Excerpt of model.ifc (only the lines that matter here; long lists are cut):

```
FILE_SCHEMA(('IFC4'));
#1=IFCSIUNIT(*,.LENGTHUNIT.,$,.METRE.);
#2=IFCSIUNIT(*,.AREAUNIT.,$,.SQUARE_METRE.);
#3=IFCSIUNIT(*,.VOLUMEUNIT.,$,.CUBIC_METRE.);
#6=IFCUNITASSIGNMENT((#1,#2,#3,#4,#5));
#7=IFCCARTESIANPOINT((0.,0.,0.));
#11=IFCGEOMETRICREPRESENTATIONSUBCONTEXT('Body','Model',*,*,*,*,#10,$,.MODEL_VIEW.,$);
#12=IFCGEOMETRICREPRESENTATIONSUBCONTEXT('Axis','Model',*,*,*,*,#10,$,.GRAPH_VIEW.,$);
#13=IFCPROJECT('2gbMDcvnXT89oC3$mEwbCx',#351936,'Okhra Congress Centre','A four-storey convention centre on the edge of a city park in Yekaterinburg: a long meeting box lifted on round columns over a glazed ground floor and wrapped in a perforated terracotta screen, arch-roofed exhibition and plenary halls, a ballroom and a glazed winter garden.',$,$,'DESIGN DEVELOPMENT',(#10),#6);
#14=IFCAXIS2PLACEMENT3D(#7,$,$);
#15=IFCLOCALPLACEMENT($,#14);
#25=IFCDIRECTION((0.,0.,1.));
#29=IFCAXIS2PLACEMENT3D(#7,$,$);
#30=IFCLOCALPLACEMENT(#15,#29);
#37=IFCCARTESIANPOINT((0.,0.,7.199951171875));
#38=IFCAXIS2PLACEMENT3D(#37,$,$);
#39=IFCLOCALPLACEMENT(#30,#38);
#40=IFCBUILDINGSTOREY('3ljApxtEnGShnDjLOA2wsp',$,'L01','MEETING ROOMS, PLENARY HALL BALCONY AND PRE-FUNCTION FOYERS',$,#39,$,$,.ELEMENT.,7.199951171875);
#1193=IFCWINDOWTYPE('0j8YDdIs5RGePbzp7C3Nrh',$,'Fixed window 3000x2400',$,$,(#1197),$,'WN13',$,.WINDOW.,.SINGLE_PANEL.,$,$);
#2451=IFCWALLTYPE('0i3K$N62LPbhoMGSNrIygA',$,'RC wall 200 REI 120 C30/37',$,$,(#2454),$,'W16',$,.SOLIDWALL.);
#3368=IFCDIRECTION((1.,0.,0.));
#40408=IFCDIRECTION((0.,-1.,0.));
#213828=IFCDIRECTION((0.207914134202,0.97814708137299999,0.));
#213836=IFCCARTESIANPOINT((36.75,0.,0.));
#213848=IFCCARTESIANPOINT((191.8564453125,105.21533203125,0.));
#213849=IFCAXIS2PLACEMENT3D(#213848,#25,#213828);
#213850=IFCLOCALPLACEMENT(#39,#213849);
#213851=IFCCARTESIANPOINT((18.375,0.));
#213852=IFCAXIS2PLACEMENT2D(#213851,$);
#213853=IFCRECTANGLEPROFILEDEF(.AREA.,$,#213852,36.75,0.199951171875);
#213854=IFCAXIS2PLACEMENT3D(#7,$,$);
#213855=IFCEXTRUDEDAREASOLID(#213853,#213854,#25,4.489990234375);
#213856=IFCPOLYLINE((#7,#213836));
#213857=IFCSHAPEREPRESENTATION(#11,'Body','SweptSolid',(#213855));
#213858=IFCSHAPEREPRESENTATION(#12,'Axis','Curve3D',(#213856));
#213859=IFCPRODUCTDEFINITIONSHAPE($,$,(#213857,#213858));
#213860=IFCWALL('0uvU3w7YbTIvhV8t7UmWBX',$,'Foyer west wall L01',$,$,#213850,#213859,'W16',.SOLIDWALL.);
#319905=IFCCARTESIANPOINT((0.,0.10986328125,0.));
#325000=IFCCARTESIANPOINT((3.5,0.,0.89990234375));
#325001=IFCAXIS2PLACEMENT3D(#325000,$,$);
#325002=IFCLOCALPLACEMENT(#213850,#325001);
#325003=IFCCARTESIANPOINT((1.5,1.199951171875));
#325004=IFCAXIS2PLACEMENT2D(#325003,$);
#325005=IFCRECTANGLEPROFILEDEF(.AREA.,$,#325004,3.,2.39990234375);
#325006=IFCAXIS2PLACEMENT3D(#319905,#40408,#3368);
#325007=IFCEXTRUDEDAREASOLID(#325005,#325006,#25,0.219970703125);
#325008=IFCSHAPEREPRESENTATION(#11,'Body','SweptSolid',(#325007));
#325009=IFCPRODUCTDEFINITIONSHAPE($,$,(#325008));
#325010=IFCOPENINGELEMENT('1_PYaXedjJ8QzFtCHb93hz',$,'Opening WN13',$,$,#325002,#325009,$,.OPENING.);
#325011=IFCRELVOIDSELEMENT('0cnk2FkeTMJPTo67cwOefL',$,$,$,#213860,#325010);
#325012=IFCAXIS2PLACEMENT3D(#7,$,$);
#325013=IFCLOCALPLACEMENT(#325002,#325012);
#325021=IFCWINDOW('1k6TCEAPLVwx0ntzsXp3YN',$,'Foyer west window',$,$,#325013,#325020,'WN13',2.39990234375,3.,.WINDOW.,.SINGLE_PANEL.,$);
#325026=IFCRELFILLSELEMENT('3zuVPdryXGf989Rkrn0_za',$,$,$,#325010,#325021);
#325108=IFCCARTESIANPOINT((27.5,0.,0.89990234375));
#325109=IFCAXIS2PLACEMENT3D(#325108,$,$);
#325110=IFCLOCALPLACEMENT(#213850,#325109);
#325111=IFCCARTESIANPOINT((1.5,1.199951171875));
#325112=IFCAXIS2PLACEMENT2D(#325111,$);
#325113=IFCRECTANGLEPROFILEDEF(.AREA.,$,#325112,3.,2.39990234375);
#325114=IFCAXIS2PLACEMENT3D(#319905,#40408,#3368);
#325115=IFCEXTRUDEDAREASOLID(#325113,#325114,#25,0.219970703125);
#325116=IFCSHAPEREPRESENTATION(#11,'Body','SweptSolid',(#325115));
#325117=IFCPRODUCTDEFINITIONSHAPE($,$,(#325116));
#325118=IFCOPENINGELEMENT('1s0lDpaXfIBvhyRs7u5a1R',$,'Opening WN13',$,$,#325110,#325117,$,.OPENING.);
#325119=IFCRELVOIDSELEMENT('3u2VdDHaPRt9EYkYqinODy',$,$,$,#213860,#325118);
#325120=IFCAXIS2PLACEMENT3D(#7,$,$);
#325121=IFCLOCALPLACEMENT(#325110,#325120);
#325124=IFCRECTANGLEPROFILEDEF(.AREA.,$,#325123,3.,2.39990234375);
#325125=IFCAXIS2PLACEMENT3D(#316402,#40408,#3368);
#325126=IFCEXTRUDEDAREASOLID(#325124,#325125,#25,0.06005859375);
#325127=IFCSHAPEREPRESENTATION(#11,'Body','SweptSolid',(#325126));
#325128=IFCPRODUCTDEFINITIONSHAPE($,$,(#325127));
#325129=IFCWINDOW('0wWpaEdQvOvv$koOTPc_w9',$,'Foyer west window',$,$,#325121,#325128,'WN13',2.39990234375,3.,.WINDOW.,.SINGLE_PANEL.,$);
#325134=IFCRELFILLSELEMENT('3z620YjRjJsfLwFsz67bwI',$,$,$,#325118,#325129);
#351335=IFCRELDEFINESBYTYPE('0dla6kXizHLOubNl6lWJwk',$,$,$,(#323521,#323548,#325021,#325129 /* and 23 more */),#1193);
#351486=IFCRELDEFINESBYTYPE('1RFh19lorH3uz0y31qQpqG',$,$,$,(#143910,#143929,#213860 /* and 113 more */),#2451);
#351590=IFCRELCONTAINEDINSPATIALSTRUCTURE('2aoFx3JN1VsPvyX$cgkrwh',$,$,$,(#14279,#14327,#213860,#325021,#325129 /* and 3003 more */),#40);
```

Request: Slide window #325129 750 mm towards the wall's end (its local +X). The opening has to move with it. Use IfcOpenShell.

```python
import ifcopenshell
import ifcopenshell.api.geometry
import ifcopenshell.util.placement

model = ifcopenshell.open("model.ifc")

window = model.by_guid("0wWpaEdQvOvv$koOTPc_w9")
opening = window.FillsVoids[0].RelatingOpeningElement
wall = opening.VoidsElements[0].RelatingBuildingElement

wall_matrix = ifcopenshell.util.placement.get_local_placement(wall.ObjectPlacement)
shift = wall_matrix[:3, 0] * 0.75
before = ifcopenshell.util.placement.get_local_placement(window.ObjectPlacement)[:3, 3].copy()

# The window is placed relative to its opening, so it follows when the opening moves.
matrix = ifcopenshell.util.placement.get_local_placement(opening.ObjectPlacement)
matrix[:3, 3] += shift
ifcopenshell.api.geometry.edit_object_placement(
    model, product=opening, matrix=matrix, is_si=False, should_transform_children=True
)

after = ifcopenshell.util.placement.get_local_placement(window.ObjectPlacement)[:3, 3]
print("window moved by", (after - before).round(3) + 0.0)

model.write("model-out.ifc")
```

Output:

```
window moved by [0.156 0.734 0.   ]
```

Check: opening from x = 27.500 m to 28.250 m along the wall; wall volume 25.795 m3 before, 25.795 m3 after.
